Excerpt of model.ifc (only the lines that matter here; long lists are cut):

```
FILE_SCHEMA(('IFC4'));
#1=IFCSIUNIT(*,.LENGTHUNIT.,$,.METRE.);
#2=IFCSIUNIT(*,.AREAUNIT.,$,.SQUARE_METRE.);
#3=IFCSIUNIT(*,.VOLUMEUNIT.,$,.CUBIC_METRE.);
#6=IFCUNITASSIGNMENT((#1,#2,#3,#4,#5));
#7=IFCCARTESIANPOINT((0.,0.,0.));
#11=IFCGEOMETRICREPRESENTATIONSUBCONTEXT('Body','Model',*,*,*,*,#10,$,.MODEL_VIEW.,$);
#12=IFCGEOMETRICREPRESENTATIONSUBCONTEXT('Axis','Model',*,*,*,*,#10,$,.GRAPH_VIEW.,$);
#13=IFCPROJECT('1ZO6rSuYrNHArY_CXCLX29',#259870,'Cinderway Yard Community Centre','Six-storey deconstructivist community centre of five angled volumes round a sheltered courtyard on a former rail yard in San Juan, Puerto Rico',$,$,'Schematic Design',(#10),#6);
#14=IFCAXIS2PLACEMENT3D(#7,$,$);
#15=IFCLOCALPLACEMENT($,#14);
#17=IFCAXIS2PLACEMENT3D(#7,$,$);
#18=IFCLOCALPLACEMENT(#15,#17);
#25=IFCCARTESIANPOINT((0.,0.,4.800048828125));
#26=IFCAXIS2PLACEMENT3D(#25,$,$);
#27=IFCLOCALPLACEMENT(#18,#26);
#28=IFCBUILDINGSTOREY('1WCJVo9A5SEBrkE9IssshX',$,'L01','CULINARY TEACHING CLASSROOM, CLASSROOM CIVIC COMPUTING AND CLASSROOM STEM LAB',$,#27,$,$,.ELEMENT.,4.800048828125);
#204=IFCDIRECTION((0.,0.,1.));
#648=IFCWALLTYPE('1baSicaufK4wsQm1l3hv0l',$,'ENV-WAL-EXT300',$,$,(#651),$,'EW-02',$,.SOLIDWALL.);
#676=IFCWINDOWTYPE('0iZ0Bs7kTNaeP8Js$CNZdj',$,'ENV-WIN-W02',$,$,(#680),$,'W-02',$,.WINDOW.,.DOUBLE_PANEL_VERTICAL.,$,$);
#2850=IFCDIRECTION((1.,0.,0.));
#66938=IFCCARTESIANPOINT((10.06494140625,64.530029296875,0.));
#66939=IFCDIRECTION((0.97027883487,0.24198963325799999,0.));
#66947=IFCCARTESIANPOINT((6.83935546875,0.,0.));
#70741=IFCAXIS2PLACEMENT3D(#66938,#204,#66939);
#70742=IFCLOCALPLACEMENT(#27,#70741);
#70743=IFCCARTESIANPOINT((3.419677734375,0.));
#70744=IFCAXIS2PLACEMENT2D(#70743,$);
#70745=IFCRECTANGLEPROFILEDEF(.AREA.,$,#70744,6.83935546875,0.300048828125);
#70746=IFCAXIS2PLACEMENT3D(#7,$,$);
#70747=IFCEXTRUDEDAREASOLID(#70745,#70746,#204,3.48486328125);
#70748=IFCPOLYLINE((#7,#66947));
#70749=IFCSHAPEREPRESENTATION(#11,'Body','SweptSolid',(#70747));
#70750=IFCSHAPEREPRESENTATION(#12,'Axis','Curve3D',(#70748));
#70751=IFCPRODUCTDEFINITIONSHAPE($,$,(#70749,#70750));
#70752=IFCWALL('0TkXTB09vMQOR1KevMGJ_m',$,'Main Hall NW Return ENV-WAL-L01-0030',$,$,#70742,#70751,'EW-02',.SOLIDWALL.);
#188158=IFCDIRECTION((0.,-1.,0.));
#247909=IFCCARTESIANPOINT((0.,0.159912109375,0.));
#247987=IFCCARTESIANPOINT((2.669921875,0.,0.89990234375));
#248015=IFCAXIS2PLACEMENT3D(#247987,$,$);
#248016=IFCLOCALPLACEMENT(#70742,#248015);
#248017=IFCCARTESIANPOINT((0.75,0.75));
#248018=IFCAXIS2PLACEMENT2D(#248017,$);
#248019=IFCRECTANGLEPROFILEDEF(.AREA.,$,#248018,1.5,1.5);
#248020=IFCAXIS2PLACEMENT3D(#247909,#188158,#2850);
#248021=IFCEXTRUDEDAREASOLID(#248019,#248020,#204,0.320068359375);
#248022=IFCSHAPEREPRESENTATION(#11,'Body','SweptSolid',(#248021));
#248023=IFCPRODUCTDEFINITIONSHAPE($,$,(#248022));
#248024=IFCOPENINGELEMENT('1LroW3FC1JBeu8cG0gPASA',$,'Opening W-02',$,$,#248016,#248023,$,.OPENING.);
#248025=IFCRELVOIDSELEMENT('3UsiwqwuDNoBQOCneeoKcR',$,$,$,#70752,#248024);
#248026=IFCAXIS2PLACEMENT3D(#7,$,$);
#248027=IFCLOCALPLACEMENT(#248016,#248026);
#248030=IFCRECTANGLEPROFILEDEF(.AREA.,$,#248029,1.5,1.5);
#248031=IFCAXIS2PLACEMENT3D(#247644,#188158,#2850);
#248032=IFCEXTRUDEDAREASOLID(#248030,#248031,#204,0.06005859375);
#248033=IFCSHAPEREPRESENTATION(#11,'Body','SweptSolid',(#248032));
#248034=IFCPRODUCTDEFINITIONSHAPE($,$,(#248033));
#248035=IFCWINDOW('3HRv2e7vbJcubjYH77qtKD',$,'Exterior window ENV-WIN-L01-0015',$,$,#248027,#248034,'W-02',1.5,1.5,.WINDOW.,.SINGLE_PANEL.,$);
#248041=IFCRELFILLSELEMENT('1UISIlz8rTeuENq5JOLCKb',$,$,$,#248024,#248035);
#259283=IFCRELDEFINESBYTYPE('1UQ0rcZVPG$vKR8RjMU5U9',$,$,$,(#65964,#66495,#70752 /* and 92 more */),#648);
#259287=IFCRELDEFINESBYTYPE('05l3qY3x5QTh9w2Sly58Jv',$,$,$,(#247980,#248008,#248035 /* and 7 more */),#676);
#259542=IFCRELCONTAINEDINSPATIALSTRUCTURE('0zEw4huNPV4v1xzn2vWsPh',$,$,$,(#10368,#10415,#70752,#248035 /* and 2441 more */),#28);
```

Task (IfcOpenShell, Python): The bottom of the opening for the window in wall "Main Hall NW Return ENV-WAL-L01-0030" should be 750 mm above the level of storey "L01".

```python
import numpy as np
import ifcopenshell
import ifcopenshell.api.geometry
import ifcopenshell.geom
import ifcopenshell.util.element
import ifcopenshell.util.placement
import ifcopenshell.util.shape
import ifcopenshell.util.unit

model = ifcopenshell.open("model.ifc")
unit_scale = ifcopenshell.util.unit.calculate_unit_scale(model)

window = model.by_id(248035)
opening = window.FillsVoids[0].RelatingOpeningElement
storey = ifcopenshell.util.element.get_container(window, ifc_class="IfcBuildingStorey")
level = ifcopenshell.util.placement.get_local_placement(storey.ObjectPlacement)[2, 3]

# The opening's origin need not be at the sill, so measure its lowest point.
shape = ifcopenshell.geom.create_shape(ifcopenshell.geom.settings(), opening)
bottom = ifcopenshell.util.shape.get_shape_bottom_elevation(shape, shape.geometry) / unit_scale
dz = level + 0.75 / unit_scale - bottom

shift = np.array([0.0, 0.0, dz])
# The window is placed relative to its opening, so it follows when the opening moves.
matrix = ifcopenshell.util.placement.get_local_placement(opening.ObjectPlacement)
matrix[:3, 3] += shift
ifcopenshell.api.geometry.edit_object_placement(
    model, product=opening, matrix=matrix, is_si=False, should_transform_children=True
)

print(f"moved by {dz * unit_scale:+.3f} m")

model.write("model_rev.ifc")
```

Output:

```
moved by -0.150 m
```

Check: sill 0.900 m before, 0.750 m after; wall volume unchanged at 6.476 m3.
